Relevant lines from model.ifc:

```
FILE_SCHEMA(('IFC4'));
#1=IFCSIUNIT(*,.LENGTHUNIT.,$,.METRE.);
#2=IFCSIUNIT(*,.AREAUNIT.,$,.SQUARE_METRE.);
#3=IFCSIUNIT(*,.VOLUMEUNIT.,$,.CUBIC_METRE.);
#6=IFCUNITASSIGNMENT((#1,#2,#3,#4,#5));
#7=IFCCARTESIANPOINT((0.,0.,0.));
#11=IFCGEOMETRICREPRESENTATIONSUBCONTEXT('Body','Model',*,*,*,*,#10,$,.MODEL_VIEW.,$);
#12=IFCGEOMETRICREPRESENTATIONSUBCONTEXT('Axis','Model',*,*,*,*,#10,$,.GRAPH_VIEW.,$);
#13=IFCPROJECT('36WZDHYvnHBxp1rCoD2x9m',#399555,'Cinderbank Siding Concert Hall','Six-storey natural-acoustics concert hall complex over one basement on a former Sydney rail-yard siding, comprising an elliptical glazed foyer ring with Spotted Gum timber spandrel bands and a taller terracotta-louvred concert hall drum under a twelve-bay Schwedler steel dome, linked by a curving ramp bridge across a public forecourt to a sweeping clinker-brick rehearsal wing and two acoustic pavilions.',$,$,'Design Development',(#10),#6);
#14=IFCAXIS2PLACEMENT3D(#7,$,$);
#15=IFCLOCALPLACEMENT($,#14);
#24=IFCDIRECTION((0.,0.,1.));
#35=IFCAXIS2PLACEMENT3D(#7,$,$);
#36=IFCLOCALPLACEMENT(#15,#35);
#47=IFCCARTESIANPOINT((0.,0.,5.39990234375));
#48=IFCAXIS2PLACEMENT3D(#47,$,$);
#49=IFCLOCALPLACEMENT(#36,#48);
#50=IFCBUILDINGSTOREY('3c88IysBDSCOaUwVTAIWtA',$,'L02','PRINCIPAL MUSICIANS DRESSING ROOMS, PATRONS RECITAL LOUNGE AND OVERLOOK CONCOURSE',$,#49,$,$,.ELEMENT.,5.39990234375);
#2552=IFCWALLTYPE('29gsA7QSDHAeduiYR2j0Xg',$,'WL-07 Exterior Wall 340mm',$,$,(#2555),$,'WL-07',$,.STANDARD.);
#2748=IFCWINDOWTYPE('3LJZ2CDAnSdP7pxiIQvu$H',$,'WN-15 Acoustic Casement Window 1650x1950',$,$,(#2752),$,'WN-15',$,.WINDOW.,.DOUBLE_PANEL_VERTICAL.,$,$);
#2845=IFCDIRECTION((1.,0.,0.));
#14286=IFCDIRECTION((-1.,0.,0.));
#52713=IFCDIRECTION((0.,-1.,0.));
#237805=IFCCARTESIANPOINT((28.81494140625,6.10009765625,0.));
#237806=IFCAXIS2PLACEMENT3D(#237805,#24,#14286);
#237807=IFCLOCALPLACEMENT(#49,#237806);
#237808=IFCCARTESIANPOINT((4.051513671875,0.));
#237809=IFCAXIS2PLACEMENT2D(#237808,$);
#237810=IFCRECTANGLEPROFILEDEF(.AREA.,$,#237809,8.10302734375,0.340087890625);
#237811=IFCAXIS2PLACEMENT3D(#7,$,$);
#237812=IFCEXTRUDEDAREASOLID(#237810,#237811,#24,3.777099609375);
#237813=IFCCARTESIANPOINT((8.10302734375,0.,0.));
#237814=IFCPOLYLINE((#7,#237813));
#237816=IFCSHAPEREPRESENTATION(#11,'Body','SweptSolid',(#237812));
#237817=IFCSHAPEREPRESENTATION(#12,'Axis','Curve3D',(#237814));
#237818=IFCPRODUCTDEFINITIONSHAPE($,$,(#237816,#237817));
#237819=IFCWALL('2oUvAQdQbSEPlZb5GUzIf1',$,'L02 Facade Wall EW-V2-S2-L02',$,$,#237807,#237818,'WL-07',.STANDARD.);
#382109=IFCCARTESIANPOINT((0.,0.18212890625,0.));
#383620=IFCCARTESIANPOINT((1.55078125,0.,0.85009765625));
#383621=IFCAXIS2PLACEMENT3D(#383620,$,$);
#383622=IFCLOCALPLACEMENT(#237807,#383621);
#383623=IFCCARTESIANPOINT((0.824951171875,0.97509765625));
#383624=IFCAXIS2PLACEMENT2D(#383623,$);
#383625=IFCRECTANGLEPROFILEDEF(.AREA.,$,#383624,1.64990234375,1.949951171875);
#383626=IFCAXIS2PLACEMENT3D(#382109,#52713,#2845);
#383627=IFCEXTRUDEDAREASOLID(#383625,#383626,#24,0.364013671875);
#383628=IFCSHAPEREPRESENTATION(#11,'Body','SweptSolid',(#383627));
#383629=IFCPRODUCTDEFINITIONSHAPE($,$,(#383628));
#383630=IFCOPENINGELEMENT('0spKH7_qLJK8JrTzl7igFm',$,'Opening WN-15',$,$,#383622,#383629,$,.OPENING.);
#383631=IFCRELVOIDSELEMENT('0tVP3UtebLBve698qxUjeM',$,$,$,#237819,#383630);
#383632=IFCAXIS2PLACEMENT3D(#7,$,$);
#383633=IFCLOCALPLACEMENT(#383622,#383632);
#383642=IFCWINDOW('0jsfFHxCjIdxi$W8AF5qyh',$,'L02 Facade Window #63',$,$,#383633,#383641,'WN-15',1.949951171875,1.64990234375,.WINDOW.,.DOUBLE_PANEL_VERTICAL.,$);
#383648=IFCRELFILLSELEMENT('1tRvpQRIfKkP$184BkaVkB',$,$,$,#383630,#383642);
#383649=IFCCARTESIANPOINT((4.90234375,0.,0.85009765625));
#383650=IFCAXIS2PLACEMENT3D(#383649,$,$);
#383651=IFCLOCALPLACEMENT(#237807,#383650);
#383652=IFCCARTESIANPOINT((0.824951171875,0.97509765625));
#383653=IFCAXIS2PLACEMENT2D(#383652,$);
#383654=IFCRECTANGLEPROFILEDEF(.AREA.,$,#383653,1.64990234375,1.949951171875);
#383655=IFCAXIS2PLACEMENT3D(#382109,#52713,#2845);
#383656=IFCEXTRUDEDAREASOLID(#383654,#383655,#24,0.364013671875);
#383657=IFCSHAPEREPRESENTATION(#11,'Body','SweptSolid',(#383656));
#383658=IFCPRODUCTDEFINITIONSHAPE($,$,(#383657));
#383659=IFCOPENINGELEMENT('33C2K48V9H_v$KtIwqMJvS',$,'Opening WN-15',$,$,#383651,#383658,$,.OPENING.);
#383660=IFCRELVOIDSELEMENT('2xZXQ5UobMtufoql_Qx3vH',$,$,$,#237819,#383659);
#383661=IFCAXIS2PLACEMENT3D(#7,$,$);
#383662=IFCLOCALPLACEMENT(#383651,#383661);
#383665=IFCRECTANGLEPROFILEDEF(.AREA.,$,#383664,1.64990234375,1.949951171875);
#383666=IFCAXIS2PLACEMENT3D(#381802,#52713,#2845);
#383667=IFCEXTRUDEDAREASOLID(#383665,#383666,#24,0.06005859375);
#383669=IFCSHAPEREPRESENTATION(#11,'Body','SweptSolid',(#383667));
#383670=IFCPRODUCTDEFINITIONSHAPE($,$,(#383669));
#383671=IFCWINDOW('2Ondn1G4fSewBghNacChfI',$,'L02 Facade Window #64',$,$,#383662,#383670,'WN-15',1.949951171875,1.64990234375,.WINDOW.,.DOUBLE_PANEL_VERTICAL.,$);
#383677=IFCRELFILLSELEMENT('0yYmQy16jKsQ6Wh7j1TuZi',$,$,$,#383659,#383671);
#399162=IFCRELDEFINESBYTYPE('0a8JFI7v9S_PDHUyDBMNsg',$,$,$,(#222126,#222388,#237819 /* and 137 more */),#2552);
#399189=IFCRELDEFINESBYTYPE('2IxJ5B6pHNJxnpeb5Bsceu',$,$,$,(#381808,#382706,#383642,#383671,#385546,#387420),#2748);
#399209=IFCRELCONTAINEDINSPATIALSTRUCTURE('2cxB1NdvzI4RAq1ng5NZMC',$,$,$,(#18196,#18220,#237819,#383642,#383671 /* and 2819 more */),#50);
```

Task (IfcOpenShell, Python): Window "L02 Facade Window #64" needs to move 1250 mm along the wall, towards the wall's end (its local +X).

```python
import ifcopenshell
import ifcopenshell.api.geometry
import ifcopenshell.util.placement
import ifcopenshell.util.unit

model = ifcopenshell.open("model.ifc")
unit_scale = ifcopenshell.util.unit.calculate_unit_scale(model)

window = model.by_guid("2Ondn1G4fSewBghNacChfI")
opening = window.FillsVoids[0].RelatingOpeningElement
wall = opening.VoidsElements[0].RelatingBuildingElement

wall_matrix = ifcopenshell.util.placement.get_local_placement(wall.ObjectPlacement)
shift = wall_matrix[:3, 0] * 1.25 / unit_scale
before = ifcopenshell.util.placement.get_local_placement(window.ObjectPlacement)[:3, 3].copy()

# The window is placed relative to its opening, so it follows when the opening moves.
matrix = ifcopenshell.util.placement.get_local_placement(opening.ObjectPlacement)
matrix[:3, 3] += shift
ifcopenshell.api.geometry.edit_object_placement(
    model, product=opening, matrix=matrix, is_si=False, should_transform_children=True
)

after = ifcopenshell.util.placement.get_local_placement(window.ObjectPlacement)[:3, 3]
print("window moved by", (after - before).round(3) + 0.0)

model.write("model-out.ifc")
```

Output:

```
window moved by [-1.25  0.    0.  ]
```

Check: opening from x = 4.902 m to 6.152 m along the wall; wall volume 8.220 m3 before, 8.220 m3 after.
